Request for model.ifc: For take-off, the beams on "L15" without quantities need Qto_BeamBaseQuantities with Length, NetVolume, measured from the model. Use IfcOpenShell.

First a look at what the model holds.

```python
import ifcopenshell
import ifcopenshell.util.element
import ifcopenshell.util.unit

model = ifcopenshell.open("model.ifc")
print(model.schema)
for unit_type in ("LENGTHUNIT", "AREAUNIT", "VOLUMEUNIT"):
    print(unit_type, ifcopenshell.util.unit.calculate_unit_scale(model, unit_type))
storey = next(s for s in model.by_type("IfcBuildingStorey") if s.Name == "L15")
beams = [e for e in ifcopenshell.util.element.get_decomposition(storey) if e.is_a("IfcBeam")]
for e in sorted(beams, key=lambda e: e.id()):
    print(e.id(), e.is_a(), e.Name, list(ifcopenshell.util.element.get_psets(e, qtos_only=True)), sep=" | ")
```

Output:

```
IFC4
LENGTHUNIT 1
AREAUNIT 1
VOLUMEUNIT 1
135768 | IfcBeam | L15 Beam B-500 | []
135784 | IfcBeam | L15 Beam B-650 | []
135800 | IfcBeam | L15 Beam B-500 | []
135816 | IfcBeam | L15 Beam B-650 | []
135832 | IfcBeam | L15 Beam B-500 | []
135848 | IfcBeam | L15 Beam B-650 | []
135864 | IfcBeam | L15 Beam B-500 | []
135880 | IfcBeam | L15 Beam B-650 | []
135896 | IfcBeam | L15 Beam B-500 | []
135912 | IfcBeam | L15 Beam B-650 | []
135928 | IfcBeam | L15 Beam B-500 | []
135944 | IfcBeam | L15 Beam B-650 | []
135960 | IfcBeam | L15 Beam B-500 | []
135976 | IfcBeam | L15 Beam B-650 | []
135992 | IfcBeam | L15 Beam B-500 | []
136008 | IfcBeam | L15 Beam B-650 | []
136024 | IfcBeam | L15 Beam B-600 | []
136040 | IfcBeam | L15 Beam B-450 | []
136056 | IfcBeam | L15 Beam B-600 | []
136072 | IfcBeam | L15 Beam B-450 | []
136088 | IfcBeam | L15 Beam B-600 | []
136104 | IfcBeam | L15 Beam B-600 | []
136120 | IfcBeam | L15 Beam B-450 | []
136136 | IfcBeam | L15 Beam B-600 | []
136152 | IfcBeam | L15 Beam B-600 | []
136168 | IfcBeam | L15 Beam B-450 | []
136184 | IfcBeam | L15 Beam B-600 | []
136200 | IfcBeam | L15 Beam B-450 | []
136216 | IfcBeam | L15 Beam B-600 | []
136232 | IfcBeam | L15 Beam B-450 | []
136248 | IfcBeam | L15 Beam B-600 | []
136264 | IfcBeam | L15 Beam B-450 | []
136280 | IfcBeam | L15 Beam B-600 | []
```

```python
import ifcopenshell
import ifcopenshell.api.pset
import ifcopenshell.geom
import ifcopenshell.util.element
import ifcopenshell.util.shape
import ifcopenshell.util.unit

model = ifcopenshell.open("model.ifc")
unit_scale = ifcopenshell.util.unit.calculate_unit_scale(model)
volume_scale = ifcopenshell.util.unit.calculate_unit_scale(model, "VOLUMEUNIT")
settings = ifcopenshell.geom.settings()

storey = next(s for s in model.by_type("IfcBuildingStorey") if s.Name == "L15")
beams = [e for e in ifcopenshell.util.element.get_decomposition(storey) if e.is_a("IfcBeam")]

for e in sorted(beams, key=lambda e: e.id()):
    if ifcopenshell.util.element.get_psets(e, qtos_only=True, should_inherit=False):
        continue
    # Geometry comes back in metres, in the element's own axes.
    shape = ifcopenshell.geom.create_shape(settings, e)
    values = {
        "Length": ifcopenshell.util.shape.get_max_xyz(shape.geometry) / unit_scale,
        "NetVolume": ifcopenshell.util.shape.get_volume(shape.geometry) / volume_scale,
    }
    qto = ifcopenshell.api.pset.add_qto(model, product=e, name="Qto_BeamBaseQuantities")
    ifcopenshell.api.pset.edit_qto(model, qto=qto, properties=values)
    print(e.id(), {k: round(v, 3) for k, v in values.items()})

model.write("model-out.ifc")
```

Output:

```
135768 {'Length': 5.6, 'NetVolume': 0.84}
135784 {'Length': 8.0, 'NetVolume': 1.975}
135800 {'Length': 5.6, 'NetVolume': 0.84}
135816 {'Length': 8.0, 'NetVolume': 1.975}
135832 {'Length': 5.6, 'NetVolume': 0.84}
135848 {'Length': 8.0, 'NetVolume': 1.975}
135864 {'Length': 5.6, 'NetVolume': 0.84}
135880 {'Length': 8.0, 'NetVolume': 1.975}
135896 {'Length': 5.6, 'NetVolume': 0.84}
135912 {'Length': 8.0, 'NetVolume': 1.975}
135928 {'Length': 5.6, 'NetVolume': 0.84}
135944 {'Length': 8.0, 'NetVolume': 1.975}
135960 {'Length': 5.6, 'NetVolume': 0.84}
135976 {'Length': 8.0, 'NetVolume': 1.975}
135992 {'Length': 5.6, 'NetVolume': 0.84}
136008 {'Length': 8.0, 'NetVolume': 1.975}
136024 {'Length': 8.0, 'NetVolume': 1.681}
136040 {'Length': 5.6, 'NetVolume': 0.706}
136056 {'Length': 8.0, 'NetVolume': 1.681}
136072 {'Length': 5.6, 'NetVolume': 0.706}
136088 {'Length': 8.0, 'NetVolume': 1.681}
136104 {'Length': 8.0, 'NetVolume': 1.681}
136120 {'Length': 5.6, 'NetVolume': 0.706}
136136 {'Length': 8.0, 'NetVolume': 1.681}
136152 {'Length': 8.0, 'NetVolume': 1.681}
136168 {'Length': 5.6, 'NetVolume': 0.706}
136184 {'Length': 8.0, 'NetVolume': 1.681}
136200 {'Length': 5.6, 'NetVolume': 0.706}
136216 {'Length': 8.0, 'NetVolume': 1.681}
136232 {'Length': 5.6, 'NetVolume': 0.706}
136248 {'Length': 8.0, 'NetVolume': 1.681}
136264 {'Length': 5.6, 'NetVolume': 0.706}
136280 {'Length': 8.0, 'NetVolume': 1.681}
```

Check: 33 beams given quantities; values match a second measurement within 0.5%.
